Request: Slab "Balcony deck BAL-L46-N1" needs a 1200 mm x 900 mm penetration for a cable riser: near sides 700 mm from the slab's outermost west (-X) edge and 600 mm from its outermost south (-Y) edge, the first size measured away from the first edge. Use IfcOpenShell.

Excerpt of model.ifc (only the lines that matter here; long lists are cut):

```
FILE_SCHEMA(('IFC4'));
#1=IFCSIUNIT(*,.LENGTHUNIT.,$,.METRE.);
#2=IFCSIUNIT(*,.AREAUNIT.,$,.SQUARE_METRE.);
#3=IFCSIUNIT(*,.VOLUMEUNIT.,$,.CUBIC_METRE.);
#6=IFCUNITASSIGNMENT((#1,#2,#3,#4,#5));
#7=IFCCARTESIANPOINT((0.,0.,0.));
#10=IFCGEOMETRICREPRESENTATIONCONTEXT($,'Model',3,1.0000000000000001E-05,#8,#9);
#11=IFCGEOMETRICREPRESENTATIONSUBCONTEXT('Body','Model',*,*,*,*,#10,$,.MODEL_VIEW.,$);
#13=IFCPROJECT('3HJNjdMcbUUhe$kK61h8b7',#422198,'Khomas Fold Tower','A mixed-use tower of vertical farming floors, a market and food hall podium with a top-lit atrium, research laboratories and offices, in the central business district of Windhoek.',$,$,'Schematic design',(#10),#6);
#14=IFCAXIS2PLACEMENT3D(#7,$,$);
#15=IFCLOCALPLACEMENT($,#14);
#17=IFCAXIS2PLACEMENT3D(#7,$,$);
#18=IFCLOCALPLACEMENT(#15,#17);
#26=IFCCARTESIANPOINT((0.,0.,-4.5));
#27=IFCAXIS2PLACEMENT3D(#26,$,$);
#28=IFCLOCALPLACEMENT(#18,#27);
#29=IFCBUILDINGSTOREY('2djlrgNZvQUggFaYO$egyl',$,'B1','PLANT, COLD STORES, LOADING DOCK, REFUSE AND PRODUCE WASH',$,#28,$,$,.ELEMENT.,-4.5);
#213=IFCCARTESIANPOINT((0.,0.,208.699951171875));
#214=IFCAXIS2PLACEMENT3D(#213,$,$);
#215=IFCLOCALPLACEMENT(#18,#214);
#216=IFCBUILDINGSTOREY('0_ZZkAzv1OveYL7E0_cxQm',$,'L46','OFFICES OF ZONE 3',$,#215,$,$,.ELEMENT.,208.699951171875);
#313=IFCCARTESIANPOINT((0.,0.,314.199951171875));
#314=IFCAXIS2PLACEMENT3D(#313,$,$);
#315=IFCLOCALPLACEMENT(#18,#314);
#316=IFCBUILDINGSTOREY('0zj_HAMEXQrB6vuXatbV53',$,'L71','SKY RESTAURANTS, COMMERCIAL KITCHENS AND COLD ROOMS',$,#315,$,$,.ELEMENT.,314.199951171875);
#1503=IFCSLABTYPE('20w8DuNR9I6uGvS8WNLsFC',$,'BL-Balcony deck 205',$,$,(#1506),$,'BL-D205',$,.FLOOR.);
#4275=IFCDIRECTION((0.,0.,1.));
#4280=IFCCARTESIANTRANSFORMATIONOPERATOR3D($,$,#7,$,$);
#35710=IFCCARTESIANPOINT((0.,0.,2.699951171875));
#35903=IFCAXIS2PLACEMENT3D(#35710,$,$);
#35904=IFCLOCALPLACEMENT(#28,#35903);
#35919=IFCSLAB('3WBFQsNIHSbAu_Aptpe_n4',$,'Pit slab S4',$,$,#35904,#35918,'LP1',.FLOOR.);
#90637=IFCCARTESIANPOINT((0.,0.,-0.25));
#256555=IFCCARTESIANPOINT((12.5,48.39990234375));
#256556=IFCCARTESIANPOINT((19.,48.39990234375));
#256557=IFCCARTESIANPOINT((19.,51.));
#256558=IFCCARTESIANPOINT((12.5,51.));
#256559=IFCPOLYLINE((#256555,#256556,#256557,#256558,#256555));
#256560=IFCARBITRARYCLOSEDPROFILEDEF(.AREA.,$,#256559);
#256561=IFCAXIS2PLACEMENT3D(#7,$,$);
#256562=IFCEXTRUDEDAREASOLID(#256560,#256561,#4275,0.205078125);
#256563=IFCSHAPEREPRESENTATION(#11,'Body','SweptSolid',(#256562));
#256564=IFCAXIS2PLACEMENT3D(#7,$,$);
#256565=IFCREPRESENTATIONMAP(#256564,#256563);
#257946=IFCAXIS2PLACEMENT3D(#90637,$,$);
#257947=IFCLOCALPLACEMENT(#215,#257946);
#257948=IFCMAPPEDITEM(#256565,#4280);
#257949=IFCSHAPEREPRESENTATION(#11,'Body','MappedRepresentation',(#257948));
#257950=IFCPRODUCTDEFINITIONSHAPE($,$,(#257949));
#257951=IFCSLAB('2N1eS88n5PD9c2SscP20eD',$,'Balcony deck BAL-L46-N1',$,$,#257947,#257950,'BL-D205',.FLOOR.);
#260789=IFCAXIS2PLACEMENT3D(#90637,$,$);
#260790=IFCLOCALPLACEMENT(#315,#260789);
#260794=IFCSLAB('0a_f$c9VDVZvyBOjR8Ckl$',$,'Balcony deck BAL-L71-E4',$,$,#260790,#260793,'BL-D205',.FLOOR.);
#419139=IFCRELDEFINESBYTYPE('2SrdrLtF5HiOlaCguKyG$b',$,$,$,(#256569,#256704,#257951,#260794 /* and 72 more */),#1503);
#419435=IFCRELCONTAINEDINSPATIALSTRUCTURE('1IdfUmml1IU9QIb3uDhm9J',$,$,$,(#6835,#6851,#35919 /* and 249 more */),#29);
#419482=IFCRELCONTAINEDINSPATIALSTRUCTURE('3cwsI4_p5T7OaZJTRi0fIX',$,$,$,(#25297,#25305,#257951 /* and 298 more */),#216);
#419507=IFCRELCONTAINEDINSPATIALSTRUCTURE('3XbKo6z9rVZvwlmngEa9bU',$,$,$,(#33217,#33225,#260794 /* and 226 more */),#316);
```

```python
import numpy as np
import ifcopenshell
import ifcopenshell.api.feature
import ifcopenshell.api.geometry
import ifcopenshell.api.root
import ifcopenshell.geom
import ifcopenshell.util.placement
import ifcopenshell.util.representation
import ifcopenshell.util.shape
import ifcopenshell.util.unit

model = ifcopenshell.open("model.ifc")
unit_scale = ifcopenshell.util.unit.calculate_unit_scale(model)
settings = ifcopenshell.geom.settings()


def volume(element):
    """Net volume in cubic metres, openings subtracted."""
    shape = ifcopenshell.geom.create_shape(settings, element)
    return ifcopenshell.util.shape.get_volume(shape.geometry)


slab = model.by_id(257951)
before = volume(slab)

# Extent in the slab's own axes, in metres. The edges named are its -X and -Y sides.
slab_shape = ifcopenshell.geom.create_shape(settings, slab)
vertices = ifcopenshell.util.shape.get_vertices(slab_shape.geometry)
x_min, y_min, bottom = vertices.min(axis=0)
top = vertices[:, 2].max()

opening = ifcopenshell.api.root.create_entity(model, ifc_class="IfcOpeningElement", name="Cable riser opening", predefined_type="OPENING")
context = ifcopenshell.util.representation.get_context(model, "Model", "Body", "MODEL_VIEW")
width, depth = 1.2, 0.9
outline = [(0.0, 0.0), (width, 0.0), (width, depth), (0.0, depth), (0.0, 0.0)]
# Overshoot both faces by 50 mm so the cut is clean.
shape = ifcopenshell.api.geometry.add_slab_representation(
    model, context=context, depth=top - bottom + 0.1, polyline=outline
)
ifcopenshell.api.geometry.assign_representation(model, product=opening, representation=shape)

matrix = ifcopenshell.util.placement.get_local_placement(slab.ObjectPlacement)
matrix[:, 3] = matrix @ np.append(np.array([x_min + 0.7, y_min + 0.6, bottom - 0.05]) / unit_scale, 1.0)
ifcopenshell.api.geometry.edit_object_placement(model, product=opening, matrix=matrix, is_si=False)
ifcopenshell.api.feature.add_feature(model, feature=opening, element=slab)

after = volume(slab)

print(f"slab volume {before:.3f} -> {after:.3f} m3")

model.write("model-out.ifc")
```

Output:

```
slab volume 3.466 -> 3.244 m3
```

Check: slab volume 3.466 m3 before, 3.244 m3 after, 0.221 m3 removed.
